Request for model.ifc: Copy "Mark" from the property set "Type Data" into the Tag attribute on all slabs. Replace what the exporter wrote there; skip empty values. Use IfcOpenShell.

First a look at what the model holds.

```python
import ifcopenshell
import ifcopenshell.util.element

model = ifcopenshell.open("model.ifc")
print(model.schema)
slabs = model.by_type("IfcSlab")
print(len(slabs), "slabs")
for e in slabs[:8]:
    source = ifcopenshell.util.element.get_pset(e, "Type Data", "Mark")
    target = e.Tag
    print(e.id(), repr(source), repr(target), sep=" | ")
```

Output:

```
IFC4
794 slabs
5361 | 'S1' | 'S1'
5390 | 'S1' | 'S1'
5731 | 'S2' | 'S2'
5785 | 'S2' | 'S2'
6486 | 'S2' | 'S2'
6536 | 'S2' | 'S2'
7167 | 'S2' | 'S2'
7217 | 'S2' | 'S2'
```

```python
import ifcopenshell
import ifcopenshell.util.element

model = ifcopenshell.open("model.ifc")

count = 0
for e in model.by_type("IfcSlab"):
    value = ifcopenshell.util.element.get_pset(e, "Type Data", "Mark")
    current = e.Tag
    if not value or not value.strip() or current == value:
        continue
    e.Tag = value
    count += 1

print(count, "slabs updated")

model.write("model-out.ifc")
```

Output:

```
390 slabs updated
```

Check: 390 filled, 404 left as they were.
